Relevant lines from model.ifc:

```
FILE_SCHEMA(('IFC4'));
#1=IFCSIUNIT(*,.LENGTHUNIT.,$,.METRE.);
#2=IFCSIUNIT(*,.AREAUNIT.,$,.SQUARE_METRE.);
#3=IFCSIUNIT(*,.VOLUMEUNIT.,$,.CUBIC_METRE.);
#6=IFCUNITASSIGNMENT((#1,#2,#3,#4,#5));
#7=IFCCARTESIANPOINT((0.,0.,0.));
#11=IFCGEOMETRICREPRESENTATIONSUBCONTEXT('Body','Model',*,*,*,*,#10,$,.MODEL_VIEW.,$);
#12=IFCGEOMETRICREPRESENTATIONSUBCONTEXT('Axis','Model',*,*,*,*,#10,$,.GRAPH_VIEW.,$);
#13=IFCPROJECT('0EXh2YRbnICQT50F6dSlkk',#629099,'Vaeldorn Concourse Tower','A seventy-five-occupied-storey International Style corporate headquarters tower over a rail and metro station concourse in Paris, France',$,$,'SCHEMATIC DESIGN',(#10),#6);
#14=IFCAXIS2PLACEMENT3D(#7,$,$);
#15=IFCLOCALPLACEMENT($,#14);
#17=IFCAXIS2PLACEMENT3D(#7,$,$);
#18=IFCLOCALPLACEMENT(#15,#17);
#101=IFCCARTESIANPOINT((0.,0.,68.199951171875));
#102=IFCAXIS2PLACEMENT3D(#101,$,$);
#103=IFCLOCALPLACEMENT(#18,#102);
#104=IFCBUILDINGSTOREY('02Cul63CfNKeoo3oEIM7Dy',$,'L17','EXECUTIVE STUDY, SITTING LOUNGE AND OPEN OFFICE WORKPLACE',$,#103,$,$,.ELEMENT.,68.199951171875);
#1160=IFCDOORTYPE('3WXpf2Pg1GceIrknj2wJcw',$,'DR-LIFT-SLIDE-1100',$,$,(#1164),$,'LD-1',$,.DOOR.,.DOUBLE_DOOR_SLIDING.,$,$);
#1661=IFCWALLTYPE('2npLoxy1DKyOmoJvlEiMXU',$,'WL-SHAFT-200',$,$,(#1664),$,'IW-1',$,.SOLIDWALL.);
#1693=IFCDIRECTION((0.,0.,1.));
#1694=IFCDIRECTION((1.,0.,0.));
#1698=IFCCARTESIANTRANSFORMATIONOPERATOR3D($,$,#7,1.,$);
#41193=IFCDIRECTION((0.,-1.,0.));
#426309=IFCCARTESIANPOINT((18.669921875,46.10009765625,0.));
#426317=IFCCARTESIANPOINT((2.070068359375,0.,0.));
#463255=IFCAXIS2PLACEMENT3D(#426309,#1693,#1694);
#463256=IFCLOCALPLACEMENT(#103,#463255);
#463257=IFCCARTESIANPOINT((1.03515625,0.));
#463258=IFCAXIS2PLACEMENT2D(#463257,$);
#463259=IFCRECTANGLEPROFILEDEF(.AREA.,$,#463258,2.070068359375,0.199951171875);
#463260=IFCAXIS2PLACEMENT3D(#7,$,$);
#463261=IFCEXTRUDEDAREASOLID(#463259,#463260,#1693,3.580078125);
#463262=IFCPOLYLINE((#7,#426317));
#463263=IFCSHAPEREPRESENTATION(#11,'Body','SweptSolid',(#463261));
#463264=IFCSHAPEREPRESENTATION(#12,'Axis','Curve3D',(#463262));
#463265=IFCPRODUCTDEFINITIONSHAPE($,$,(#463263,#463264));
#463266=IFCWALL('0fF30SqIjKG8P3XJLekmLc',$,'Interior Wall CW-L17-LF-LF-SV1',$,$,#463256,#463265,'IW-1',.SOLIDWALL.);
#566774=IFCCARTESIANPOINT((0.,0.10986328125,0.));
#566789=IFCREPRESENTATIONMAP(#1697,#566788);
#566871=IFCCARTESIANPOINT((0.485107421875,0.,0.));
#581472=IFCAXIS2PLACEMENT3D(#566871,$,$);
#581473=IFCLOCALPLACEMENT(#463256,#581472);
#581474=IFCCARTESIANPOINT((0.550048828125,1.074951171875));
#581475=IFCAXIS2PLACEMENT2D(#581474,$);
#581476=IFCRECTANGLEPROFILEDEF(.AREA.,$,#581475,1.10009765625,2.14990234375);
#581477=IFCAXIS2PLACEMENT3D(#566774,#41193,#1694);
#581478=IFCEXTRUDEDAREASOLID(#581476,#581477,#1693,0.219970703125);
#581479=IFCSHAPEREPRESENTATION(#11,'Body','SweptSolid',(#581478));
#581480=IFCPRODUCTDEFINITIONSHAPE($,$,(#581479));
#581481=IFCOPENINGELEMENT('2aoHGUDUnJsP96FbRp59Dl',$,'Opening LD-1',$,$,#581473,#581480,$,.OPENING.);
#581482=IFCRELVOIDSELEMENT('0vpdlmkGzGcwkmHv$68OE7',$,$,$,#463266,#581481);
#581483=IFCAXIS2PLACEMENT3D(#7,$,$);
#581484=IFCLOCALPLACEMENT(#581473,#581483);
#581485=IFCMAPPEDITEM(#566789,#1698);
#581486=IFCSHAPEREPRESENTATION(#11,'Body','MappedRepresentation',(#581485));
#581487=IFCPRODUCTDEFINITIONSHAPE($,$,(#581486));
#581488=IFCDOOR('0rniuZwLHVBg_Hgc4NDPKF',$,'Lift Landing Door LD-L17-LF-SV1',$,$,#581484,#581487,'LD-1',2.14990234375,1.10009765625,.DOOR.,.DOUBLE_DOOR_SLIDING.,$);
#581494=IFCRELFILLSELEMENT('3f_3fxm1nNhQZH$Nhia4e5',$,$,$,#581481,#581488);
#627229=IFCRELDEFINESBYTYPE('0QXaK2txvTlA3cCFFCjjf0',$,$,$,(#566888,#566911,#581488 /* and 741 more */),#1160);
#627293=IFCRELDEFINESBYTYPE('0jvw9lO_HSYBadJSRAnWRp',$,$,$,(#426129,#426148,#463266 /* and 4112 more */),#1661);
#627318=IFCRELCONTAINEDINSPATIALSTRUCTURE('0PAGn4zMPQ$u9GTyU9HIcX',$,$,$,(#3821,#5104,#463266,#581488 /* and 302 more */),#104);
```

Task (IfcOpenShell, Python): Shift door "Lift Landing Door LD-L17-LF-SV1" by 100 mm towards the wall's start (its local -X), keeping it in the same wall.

```python
import ifcopenshell
import ifcopenshell.api.geometry
import ifcopenshell.util.placement

model = ifcopenshell.open("model.ifc")

door = model.by_guid("0rniuZwLHVBg_Hgc4NDPKF")
opening = door.FillsVoids[0].RelatingOpeningElement
wall = opening.VoidsElements[0].RelatingBuildingElement

wall_matrix = ifcopenshell.util.placement.get_local_placement(wall.ObjectPlacement)
shift = wall_matrix[:3, 0] * -0.1
before = ifcopenshell.util.placement.get_local_placement(door.ObjectPlacement)[:3, 3].copy()

# The door is placed relative to its opening, so it follows when the opening moves.
matrix = ifcopenshell.util.placement.get_local_placement(opening.ObjectPlacement)
matrix[:3, 3] += shift
ifcopenshell.api.geometry.edit_object_placement(
    model, product=opening, matrix=matrix, is_si=False, should_transform_children=True
)

after = ifcopenshell.util.placement.get_local_placement(door.ObjectPlacement)[:3, 3]
print("door moved by", (after - before).round(3) + 0.0)

model.write("model_edited.ifc")
```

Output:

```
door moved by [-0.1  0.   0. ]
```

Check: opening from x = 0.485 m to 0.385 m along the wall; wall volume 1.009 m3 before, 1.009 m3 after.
